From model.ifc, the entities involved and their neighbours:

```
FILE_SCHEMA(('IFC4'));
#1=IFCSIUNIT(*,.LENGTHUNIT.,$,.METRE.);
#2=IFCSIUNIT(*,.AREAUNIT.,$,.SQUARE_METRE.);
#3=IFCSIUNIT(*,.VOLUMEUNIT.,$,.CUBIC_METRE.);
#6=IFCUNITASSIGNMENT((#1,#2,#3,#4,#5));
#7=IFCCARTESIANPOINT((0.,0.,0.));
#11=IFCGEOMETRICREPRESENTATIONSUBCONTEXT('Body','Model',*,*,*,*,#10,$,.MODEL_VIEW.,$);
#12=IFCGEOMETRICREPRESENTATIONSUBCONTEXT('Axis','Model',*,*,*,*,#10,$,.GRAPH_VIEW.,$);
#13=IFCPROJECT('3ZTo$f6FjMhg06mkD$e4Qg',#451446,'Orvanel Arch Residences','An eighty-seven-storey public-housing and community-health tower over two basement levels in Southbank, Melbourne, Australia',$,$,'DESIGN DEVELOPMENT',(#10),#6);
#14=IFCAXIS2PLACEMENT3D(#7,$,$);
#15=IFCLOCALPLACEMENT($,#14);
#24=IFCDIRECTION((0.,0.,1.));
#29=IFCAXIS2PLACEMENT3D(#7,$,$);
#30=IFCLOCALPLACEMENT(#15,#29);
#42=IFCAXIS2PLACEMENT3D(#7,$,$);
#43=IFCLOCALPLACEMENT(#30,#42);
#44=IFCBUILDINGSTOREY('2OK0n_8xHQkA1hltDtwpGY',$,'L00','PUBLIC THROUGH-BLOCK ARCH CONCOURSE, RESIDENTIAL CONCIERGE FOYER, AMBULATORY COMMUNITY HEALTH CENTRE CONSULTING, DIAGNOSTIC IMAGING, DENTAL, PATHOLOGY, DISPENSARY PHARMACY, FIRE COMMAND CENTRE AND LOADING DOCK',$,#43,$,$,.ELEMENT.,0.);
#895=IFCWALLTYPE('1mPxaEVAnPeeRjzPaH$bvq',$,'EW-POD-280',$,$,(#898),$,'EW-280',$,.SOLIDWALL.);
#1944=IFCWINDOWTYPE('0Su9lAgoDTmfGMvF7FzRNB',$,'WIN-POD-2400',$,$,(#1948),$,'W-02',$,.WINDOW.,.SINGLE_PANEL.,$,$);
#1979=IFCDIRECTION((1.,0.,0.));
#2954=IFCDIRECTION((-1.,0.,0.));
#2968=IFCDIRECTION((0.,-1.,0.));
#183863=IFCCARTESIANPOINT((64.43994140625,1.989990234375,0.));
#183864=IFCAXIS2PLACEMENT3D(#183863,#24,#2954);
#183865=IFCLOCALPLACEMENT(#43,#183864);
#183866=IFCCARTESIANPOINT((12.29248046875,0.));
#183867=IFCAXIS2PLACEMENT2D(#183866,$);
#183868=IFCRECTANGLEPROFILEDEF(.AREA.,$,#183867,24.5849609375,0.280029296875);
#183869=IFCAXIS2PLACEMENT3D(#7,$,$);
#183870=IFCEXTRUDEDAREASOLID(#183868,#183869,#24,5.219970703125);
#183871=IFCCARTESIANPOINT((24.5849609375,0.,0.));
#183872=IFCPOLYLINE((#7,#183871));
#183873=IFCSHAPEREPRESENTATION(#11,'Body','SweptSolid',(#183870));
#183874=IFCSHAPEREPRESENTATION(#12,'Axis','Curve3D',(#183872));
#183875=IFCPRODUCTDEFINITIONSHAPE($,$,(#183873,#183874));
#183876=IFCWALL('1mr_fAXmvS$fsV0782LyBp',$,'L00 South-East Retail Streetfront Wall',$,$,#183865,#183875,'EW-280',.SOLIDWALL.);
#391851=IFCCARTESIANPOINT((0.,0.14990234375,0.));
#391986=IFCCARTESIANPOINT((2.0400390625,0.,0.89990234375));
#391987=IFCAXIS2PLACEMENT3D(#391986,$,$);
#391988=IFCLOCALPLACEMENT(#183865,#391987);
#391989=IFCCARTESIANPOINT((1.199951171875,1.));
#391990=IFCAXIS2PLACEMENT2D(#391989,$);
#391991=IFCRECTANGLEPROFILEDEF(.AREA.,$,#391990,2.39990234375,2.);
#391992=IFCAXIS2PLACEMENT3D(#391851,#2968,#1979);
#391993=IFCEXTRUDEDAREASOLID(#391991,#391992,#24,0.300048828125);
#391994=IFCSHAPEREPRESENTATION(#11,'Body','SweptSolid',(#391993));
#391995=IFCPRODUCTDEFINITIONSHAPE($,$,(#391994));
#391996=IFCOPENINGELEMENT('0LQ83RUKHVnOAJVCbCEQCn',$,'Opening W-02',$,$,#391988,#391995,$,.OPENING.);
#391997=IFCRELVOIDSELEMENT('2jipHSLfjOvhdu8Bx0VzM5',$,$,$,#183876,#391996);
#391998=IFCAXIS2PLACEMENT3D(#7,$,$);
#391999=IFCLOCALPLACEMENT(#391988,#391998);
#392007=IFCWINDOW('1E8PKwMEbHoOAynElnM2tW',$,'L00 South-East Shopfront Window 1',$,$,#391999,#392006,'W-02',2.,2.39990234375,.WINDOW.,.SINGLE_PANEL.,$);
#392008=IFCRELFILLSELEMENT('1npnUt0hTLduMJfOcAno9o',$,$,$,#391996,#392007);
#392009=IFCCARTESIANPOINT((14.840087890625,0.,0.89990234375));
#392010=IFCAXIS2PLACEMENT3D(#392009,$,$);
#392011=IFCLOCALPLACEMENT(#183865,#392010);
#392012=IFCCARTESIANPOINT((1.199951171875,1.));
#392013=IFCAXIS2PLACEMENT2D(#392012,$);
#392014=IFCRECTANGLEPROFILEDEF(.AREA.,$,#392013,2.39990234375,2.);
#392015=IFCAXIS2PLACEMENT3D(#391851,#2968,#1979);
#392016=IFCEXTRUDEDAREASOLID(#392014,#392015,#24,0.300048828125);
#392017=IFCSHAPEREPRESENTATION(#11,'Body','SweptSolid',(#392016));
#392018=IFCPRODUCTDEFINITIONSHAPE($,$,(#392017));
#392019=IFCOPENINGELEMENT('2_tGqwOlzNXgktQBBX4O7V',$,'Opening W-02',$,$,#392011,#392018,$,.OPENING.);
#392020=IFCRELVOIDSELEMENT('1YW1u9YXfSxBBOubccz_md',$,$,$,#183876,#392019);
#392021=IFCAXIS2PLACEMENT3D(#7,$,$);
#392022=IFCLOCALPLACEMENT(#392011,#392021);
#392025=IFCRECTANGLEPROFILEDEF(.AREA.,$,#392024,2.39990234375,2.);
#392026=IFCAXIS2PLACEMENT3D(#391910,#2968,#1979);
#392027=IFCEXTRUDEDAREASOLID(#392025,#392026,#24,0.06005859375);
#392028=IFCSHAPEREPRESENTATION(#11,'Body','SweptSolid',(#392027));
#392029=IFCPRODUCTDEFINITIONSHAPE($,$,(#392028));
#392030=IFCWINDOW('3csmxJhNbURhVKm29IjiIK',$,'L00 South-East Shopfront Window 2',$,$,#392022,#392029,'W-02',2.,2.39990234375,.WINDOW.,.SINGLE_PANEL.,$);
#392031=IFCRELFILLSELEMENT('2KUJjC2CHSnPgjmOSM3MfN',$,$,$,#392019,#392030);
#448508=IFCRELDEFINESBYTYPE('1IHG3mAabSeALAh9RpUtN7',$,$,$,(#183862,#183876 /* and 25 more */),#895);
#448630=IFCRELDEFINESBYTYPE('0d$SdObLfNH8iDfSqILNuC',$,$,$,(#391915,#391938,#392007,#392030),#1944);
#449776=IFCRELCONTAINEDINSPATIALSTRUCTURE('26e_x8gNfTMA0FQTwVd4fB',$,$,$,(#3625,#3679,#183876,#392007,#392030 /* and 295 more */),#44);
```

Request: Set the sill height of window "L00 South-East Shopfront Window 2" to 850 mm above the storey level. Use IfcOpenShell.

```python
import numpy as np
import ifcopenshell
import ifcopenshell.api.geometry
import ifcopenshell.geom
import ifcopenshell.util.element
import ifcopenshell.util.placement
import ifcopenshell.util.shape
import ifcopenshell.util.unit

model = ifcopenshell.open("model.ifc")
unit_scale = ifcopenshell.util.unit.calculate_unit_scale(model)

window = model.by_id(392030)
opening = window.FillsVoids[0].RelatingOpeningElement
storey = ifcopenshell.util.element.get_container(window, ifc_class="IfcBuildingStorey")
level = ifcopenshell.util.placement.get_local_placement(storey.ObjectPlacement)[2, 3]

# The opening's origin need not be at the sill, so measure its lowest point.
shape = ifcopenshell.geom.create_shape(ifcopenshell.geom.settings(), opening)
bottom = ifcopenshell.util.shape.get_shape_bottom_elevation(shape, shape.geometry) / unit_scale
dz = level + 0.85 - bottom

shift = np.array([0.0, 0.0, dz])
# The window is placed relative to its opening, so it follows when the opening moves.
matrix = ifcopenshell.util.placement.get_local_placement(opening.ObjectPlacement)
matrix[:3, 3] += shift
ifcopenshell.api.geometry.edit_object_placement(
    model, product=opening, matrix=matrix, is_si=False, should_transform_children=True
)

print(f"moved by {dz * unit_scale:+.3f} m")

model.write("model_edited.ifc")
```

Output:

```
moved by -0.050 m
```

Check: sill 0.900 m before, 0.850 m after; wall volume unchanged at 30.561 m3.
